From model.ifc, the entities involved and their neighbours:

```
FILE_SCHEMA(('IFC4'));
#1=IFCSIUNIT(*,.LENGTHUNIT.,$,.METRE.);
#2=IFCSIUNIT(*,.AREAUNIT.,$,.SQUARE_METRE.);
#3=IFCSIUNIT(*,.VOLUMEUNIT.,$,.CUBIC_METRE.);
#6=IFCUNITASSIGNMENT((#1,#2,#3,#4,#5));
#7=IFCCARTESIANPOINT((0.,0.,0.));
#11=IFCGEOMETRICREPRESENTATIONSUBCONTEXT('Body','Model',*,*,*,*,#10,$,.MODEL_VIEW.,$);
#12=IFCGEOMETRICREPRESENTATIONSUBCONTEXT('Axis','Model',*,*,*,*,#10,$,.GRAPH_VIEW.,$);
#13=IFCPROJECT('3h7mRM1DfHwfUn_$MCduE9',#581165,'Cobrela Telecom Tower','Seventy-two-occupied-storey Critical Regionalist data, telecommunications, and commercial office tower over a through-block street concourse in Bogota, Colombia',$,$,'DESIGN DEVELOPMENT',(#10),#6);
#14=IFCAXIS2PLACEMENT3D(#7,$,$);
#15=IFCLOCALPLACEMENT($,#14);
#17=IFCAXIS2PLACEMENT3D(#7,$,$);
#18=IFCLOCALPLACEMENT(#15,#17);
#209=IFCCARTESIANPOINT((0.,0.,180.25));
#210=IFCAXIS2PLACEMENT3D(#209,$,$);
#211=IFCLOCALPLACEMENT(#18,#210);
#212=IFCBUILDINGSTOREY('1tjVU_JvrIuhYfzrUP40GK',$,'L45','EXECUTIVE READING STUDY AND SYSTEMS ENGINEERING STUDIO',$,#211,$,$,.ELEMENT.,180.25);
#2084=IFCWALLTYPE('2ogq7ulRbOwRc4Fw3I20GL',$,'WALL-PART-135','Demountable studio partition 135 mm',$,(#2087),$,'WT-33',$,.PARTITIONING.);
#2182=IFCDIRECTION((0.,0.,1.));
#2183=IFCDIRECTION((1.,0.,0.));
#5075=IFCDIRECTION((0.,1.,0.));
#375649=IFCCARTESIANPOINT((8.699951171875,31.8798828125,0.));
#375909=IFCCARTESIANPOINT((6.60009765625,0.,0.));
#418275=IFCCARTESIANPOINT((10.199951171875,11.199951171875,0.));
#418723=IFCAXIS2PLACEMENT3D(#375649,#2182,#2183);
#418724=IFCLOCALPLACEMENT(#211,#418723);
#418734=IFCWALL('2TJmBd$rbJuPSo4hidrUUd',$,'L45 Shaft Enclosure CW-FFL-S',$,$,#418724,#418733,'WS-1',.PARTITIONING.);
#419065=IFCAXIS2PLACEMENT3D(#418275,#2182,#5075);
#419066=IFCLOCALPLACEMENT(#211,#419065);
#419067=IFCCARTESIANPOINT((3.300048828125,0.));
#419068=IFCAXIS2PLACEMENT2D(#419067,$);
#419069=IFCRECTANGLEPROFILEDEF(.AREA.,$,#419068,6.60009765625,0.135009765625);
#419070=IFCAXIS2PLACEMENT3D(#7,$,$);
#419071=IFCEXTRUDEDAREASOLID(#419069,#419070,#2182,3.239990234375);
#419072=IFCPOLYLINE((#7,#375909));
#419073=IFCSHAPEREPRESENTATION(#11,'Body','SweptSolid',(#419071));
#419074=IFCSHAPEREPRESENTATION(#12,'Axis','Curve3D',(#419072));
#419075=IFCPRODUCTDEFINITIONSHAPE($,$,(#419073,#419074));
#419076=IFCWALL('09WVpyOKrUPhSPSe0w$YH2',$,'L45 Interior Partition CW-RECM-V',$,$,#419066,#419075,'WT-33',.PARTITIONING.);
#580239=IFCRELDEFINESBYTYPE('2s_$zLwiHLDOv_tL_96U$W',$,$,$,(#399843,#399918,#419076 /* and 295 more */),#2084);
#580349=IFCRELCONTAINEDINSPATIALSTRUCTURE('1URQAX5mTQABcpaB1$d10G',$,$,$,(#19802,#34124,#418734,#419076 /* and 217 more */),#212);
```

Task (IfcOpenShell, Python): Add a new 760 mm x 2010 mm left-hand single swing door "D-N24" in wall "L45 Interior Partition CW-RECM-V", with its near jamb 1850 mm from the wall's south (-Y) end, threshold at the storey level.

```python
import numpy as np
import ifcopenshell
import ifcopenshell.api.feature
import ifcopenshell.api.geometry
import ifcopenshell.api.root
import ifcopenshell.api.spatial
import ifcopenshell.geom
import ifcopenshell.util.element
import ifcopenshell.util.placement
import ifcopenshell.util.representation
import ifcopenshell.util.shape
import ifcopenshell.util.unit

model = ifcopenshell.open("model.ifc")
unit_scale = ifcopenshell.util.unit.calculate_unit_scale(model)
settings = ifcopenshell.geom.settings()


def volume(element):
    """Net volume in cubic metres, openings subtracted."""
    shape = ifcopenshell.geom.create_shape(settings, element)
    return ifcopenshell.util.shape.get_volume(shape.geometry)


wall = model.by_guid("09WVpyOKrUPhSPSe0w$YH2")
storey = ifcopenshell.util.element.get_container(wall, ifc_class="IfcBuildingStorey")
context = ifcopenshell.util.representation.get_context(model, "Model", "Body", "MODEL_VIEW")
before = volume(wall)

width, height, from_end, sill = 0.76, 2.01, 1.85, 0.0  # metres

# The wall runs along its own X axis, and the end named is its -X end.
wall_shape = ifcopenshell.geom.create_shape(settings, wall)
x, y, z = ifcopenshell.util.shape.get_vertices(wall_shape.geometry).T
start = x.min() + from_end
face, thickness = float(y.min()), float(y.max() - y.min())
wall_matrix = ifcopenshell.util.placement.get_local_placement(wall.ObjectPlacement)
level = ifcopenshell.util.placement.get_local_placement(storey.ObjectPlacement)[2, 3]


def in_wall(x, y):
    """Placement at x, y metres in the wall's axes, at sill height."""
    matrix = wall_matrix.copy()
    matrix[:, 3] = wall_matrix @ np.array([x / unit_scale, y / unit_scale, 0.0, 1.0])
    matrix[2, 3] = level + sill / unit_scale
    return matrix


# Opening: a box that overshoots both wall faces by 50 mm.
opening = ifcopenshell.api.root.create_entity(model, ifc_class="IfcOpeningElement", predefined_type="OPENING")
box = ifcopenshell.api.geometry.add_wall_representation(
    model, context=context, length=width, height=height, thickness=thickness + 0.1
)
ifcopenshell.api.geometry.assign_representation(model, product=opening, representation=box)
ifcopenshell.api.geometry.edit_object_placement(model, product=opening, matrix=in_wall(start, face - 0.05), is_si=False)
ifcopenshell.api.feature.add_feature(model, feature=opening, element=wall)

door = ifcopenshell.api.root.create_entity(model, ifc_class="IfcDoor", name="D-N24", predefined_type="DOOR")
door.OverallWidth, door.OverallHeight = width / unit_scale, height / unit_scale
door.OperationType = "SINGLE_SWING_LEFT"
body = ifcopenshell.api.geometry.add_door_representation(
    model,
    context=context,
    overall_width=door.OverallWidth,
    overall_height=door.OverallHeight,
    operation_type="SINGLE_SWING_LEFT",
    lining_properties={"LiningDepth": thickness / unit_scale, "ThresholdDepth": thickness / unit_scale},
)
ifcopenshell.api.geometry.assign_representation(model, product=door, representation=body)
ifcopenshell.api.spatial.assign_container(model, products=[door], relating_structure=storey)
ifcopenshell.api.feature.add_filling(model, opening=opening, element=door)

# The lining spans the wall, so the door starts at the wall face.
ifcopenshell.api.geometry.edit_object_placement(model, product=door, matrix=in_wall(start, face), is_si=False)

after = volume(wall)

print(f"wall volume {before:.3f} -> {after:.3f} m3")

model.write("model-out.ifc")
```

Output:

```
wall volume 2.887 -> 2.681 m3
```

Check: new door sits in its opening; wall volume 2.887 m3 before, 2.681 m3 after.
